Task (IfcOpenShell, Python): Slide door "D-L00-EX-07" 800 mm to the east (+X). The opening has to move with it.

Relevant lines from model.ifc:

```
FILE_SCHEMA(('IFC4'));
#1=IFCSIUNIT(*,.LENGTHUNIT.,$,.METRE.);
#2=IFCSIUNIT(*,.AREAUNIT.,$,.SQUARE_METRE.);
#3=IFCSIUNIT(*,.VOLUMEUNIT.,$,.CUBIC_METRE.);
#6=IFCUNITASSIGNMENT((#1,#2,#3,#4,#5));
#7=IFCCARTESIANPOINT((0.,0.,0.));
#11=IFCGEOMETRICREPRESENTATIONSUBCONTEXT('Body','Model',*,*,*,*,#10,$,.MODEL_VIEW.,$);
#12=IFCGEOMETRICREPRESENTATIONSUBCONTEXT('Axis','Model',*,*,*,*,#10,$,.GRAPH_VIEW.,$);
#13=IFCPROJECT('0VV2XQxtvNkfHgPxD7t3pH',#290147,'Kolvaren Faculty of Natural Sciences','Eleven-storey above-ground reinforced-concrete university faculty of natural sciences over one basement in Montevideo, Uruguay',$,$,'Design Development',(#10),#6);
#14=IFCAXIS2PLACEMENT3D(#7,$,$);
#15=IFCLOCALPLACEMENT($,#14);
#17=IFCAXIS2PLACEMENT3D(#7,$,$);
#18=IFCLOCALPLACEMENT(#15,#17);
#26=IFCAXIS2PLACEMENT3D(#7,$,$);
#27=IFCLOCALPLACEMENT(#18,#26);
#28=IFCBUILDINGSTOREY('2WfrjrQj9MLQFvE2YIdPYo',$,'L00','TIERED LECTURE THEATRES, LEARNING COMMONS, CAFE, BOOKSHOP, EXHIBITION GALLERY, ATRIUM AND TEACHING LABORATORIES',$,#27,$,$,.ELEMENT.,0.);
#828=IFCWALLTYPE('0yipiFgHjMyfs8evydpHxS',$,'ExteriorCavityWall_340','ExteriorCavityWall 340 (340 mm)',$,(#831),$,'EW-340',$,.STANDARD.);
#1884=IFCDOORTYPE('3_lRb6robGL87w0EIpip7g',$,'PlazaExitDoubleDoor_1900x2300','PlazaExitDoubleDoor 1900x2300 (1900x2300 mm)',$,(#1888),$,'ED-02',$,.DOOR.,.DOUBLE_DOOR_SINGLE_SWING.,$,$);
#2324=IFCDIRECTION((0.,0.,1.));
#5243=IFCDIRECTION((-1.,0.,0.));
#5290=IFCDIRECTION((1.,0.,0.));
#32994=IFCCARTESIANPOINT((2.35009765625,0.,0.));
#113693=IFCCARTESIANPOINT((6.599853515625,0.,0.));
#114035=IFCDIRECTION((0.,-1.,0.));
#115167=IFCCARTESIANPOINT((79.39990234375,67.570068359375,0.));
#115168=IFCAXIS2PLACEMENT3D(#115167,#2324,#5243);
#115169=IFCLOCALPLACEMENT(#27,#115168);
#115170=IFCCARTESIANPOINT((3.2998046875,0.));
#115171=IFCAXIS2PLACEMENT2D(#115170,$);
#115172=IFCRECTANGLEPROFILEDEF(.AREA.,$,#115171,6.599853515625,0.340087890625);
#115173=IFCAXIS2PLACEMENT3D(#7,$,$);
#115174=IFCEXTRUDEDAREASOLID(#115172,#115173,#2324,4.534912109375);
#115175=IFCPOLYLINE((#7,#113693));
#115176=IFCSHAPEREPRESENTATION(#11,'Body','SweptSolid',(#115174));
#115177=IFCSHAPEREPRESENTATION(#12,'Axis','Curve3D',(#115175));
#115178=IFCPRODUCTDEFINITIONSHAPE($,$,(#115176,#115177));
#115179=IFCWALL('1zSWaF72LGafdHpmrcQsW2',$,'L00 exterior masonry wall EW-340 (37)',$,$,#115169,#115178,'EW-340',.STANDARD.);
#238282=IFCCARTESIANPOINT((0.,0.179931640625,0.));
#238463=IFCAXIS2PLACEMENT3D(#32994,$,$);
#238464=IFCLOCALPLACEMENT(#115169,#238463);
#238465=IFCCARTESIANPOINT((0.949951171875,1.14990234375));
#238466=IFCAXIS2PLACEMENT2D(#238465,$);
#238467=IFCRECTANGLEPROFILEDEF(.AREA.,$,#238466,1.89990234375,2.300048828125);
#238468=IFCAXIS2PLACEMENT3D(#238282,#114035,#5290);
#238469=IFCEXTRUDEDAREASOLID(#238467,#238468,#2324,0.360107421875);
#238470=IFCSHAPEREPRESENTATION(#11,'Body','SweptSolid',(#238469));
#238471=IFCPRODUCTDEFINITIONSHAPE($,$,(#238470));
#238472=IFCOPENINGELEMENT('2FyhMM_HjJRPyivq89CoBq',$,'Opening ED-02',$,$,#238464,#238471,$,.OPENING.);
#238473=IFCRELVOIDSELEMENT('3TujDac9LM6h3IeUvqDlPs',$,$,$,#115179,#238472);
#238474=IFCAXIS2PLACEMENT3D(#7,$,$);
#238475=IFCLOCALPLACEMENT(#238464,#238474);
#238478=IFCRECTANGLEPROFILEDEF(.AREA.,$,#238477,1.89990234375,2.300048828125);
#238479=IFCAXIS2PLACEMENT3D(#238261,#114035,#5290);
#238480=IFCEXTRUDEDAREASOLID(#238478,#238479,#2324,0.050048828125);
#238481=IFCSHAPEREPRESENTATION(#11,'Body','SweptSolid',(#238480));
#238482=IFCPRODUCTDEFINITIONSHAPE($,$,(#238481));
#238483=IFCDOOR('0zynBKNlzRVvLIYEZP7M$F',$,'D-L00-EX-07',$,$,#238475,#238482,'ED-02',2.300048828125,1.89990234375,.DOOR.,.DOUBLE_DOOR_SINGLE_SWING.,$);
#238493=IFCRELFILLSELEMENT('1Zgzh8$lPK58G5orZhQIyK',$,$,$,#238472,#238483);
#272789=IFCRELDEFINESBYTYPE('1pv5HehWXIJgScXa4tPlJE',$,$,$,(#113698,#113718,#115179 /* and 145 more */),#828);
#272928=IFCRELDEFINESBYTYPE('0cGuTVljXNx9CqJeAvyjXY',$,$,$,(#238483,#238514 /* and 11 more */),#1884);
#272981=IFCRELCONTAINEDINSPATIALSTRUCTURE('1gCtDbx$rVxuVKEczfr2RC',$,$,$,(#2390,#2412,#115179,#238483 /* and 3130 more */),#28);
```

```python
import ifcopenshell
import ifcopenshell.api.geometry
import ifcopenshell.util.placement

model = ifcopenshell.open("model.ifc")

door = model.by_id(238483)
opening = door.FillsVoids[0].RelatingOpeningElement
wall = opening.VoidsElements[0].RelatingBuildingElement

wall_matrix = ifcopenshell.util.placement.get_local_placement(wall.ObjectPlacement)
shift = wall_matrix[:3, 0] * -0.8
before = ifcopenshell.util.placement.get_local_placement(door.ObjectPlacement)[:3, 3].copy()

# The door is placed relative to its opening, so it follows when the opening moves.
matrix = ifcopenshell.util.placement.get_local_placement(opening.ObjectPlacement)
matrix[:3, 3] += shift
ifcopenshell.api.geometry.edit_object_placement(
    model, product=opening, matrix=matrix, is_si=False, should_transform_children=True
)

after = ifcopenshell.util.placement.get_local_placement(door.ObjectPlacement)[:3, 3]
print("door moved by", (after - before).round(3) + 0.0)

model.write("model_v2.ifc")
```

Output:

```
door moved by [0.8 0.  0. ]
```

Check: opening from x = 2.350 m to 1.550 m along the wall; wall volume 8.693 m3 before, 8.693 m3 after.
